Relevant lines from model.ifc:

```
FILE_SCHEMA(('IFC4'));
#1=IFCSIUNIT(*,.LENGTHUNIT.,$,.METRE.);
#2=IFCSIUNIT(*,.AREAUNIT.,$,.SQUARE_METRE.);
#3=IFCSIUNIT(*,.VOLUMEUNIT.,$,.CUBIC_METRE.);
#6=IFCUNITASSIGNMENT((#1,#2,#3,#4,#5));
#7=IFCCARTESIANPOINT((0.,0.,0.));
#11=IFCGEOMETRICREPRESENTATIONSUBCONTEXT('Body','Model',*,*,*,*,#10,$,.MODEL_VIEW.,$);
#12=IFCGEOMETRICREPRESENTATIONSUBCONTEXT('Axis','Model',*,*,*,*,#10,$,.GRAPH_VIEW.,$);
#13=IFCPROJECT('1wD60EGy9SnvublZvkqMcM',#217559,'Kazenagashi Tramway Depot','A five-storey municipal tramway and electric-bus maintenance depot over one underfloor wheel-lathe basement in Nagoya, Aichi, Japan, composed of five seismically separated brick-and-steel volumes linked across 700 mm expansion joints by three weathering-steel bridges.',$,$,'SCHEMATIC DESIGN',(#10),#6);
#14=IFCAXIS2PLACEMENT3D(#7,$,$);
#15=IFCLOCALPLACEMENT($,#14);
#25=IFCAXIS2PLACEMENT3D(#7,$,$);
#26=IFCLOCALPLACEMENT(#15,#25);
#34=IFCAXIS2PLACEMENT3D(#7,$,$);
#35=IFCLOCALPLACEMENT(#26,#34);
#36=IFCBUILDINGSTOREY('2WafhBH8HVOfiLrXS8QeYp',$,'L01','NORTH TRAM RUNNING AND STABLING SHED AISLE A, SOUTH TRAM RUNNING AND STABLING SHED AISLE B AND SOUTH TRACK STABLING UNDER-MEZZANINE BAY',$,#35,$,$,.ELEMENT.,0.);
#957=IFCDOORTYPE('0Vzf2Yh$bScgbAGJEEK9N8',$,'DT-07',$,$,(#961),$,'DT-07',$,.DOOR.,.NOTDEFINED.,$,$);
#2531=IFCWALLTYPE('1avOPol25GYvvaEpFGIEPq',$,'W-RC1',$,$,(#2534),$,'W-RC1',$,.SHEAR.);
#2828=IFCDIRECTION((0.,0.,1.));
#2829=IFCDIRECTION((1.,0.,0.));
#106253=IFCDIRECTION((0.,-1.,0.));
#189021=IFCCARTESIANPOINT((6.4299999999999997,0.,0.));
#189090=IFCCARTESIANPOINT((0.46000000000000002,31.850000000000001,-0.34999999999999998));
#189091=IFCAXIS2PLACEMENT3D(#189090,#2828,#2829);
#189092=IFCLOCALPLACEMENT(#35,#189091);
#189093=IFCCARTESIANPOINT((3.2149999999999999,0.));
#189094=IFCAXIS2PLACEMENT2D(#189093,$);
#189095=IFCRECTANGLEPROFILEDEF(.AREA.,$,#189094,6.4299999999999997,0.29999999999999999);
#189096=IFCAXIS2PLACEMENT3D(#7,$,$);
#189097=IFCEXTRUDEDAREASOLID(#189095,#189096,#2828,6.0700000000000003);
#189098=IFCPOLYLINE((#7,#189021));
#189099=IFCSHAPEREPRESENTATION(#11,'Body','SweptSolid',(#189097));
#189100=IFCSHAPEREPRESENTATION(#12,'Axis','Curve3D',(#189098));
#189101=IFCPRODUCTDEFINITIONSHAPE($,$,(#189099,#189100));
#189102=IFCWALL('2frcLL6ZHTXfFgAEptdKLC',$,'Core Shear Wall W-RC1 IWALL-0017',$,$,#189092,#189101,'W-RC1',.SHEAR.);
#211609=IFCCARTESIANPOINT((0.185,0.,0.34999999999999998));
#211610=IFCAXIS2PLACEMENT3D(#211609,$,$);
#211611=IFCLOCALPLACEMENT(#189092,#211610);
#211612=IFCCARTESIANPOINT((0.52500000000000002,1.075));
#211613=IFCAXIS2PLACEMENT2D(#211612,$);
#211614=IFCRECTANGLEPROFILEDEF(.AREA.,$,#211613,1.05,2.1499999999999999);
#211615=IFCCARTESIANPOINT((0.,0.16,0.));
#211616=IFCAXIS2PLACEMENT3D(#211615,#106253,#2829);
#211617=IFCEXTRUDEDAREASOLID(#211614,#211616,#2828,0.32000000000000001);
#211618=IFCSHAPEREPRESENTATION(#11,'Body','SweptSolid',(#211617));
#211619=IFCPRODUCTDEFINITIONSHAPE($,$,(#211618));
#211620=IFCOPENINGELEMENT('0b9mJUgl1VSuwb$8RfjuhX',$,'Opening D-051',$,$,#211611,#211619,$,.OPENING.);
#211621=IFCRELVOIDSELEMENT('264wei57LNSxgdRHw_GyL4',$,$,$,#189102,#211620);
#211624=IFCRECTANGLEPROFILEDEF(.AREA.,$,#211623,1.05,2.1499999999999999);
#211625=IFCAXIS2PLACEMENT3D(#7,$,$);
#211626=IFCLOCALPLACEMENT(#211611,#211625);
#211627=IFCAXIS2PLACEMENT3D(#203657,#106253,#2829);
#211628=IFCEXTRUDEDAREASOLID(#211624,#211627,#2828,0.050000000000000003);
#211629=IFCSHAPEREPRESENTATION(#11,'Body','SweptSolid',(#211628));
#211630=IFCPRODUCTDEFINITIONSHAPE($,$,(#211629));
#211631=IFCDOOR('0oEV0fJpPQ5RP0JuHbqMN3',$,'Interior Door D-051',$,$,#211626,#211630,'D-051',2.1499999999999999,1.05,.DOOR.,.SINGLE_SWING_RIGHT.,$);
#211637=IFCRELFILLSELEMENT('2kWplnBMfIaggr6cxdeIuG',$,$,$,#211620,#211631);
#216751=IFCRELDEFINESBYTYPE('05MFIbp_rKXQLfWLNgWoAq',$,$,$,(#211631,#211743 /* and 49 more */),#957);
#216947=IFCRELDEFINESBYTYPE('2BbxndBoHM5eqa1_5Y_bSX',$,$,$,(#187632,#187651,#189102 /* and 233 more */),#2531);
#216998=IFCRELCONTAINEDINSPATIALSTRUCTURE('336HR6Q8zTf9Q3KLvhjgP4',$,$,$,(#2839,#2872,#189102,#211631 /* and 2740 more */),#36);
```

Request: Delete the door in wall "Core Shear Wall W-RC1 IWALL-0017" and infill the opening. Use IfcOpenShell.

```python
import ifcopenshell
import ifcopenshell.api.feature
import ifcopenshell.api.root
import ifcopenshell.geom
import ifcopenshell.util.shape

model = ifcopenshell.open("model.ifc")
settings = ifcopenshell.geom.settings()


def volume(element):
    """Net volume in cubic metres, openings subtracted."""
    shape = ifcopenshell.geom.create_shape(settings, element)
    return ifcopenshell.util.shape.get_volume(shape.geometry)


door = model.by_guid("0oEV0fJpPQ5RP0JuHbqMN3")
opening = door.FillsVoids[0].RelatingOpeningElement
wall = opening.VoidsElements[0].RelatingBuildingElement
before = volume(wall)

ifcopenshell.api.root.remove_product(model, product=door)
ifcopenshell.api.feature.remove_feature(model, feature=opening)

after = volume(wall)

print(f"wall volume {before:.3f} -> {after:.3f} m3")

model.write("model_updated.ifc")
```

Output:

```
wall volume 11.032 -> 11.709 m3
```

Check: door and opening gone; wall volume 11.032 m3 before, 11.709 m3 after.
